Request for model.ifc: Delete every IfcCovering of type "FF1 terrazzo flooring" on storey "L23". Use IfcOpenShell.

First a look at what the model holds.

```python
import ifcopenshell
import ifcopenshell.util.element

model = ifcopenshell.open("model.ifc")
print(model.schema)
storey = next(s for s in model.by_type("IfcBuildingStorey") if s.Name == "L23")
coverings = [e for e in ifcopenshell.util.element.get_decomposition(storey) if e.is_a("IfcCovering")]
seen = {}
for e in coverings:
    element_type = ifcopenshell.util.element.get_type(e)
    name = element_type.Name if element_type not in (None, e) else None
    seen[name] = seen.get(name, 0) + 1
for name, count in sorted(seen.items(), key=str):
    print(count, "x", name)
```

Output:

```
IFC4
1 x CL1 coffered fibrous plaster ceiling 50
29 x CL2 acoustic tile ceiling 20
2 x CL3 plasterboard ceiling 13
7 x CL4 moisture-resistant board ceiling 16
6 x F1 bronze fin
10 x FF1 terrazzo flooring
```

```python
import ifcopenshell
import ifcopenshell.api.root
import ifcopenshell.util.element

model = ifcopenshell.open("model.ifc")

storey = next(s for s in model.by_type("IfcBuildingStorey") if s.Name == "L23")
coverings = [e for e in ifcopenshell.util.element.get_decomposition(storey) if e.is_a("IfcCovering")]
targets = [e for e in coverings if (t := ifcopenshell.util.element.get_type(e)) not in (None, e) and t.Name == "FF1 terrazzo flooring"]

for e in targets:
    ifcopenshell.api.root.remove_product(model, product=e)
print(len(targets), "removed")

model.write("model-out.ifc")
```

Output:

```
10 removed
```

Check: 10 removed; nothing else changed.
